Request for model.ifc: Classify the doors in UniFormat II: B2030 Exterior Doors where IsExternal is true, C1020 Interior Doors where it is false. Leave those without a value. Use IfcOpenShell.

First a look at what the model holds.

```python
import ifcopenshell
import ifcopenshell.util.element

model = ifcopenshell.open("model.ifc")
print(model.schema)
print("classifications:", [c.Name for c in model.by_type("IfcClassification")])
values = [ifcopenshell.util.element.get_pset(e, "Pset_DoorCommon", "IsExternal") for e in model.by_type("IfcDoor")]
for value in (True, False, None):
    print("IsExternal", value, values.count(value))
```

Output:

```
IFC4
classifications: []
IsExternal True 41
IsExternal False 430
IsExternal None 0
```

```python
import ifcopenshell
import ifcopenshell.api.classification
import ifcopenshell.util.element

model = ifcopenshell.open("model.ifc")

system = ifcopenshell.api.classification.add_classification(model, classification="UniFormat II")

doors = model.by_type("IfcDoor")
external = {e: ifcopenshell.util.element.get_pset(e, "Pset_DoorCommon", "IsExternal") for e in doors}
for flag, code, name in ((True, "B2030", "Exterior Doors"), (False, "C1020", "Interior Doors")):
    products = [e for e in doors if external[e] is flag]
    ifcopenshell.api.classification.add_reference(
        model, products=products, classification=system, identification=code, name=name
    )
    print(code, len(products))

model.write("model_updated.ifc")
```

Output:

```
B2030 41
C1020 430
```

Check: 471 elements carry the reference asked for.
